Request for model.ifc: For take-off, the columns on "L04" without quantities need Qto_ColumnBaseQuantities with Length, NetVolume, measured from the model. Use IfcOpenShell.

First a look at what the model holds.

```python
import ifcopenshell
import ifcopenshell.util.element
import ifcopenshell.util.unit

model = ifcopenshell.open("model.ifc")
print(model.schema)
for unit_type in ("LENGTHUNIT", "AREAUNIT", "VOLUMEUNIT"):
    print(unit_type, ifcopenshell.util.unit.calculate_unit_scale(model, unit_type))
storey = next(s for s in model.by_type("IfcBuildingStorey") if s.Name == "L04")
columns = [e for e in ifcopenshell.util.element.get_decomposition(storey) if e.is_a("IfcColumn")]
for e in sorted(columns, key=lambda e: e.id()):
    print(e.id(), e.is_a(), e.Name, list(ifcopenshell.util.element.get_psets(e, qtos_only=True)), sep=" | ")
```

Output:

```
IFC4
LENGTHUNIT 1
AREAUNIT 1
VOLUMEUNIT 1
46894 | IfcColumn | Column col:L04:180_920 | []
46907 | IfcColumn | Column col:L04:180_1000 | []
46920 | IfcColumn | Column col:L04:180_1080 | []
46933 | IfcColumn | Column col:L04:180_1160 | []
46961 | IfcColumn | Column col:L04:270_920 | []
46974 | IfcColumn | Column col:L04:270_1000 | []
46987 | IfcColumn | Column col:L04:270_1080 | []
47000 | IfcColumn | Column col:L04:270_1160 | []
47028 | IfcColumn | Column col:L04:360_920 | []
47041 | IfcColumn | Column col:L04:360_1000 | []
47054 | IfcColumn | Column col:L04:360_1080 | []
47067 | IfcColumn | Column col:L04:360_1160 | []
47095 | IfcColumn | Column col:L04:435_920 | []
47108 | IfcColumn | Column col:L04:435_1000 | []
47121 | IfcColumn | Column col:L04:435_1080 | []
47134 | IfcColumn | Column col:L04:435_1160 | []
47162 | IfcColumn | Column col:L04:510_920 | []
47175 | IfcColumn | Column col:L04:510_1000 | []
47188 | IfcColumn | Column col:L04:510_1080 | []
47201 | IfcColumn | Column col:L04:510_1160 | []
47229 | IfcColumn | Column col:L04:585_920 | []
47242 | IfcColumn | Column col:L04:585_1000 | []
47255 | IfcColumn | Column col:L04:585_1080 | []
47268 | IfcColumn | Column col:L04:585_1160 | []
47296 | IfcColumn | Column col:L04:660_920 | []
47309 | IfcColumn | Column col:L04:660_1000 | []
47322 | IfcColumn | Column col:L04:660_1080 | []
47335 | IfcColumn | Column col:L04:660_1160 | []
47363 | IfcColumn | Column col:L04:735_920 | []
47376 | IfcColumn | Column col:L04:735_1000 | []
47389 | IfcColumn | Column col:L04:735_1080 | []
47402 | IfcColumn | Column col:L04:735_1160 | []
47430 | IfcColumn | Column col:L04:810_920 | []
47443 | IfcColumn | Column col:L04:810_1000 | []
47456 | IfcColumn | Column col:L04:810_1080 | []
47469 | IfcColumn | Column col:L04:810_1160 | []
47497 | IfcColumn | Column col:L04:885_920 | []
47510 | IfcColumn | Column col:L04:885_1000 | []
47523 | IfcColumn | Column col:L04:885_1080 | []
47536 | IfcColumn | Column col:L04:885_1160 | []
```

```python
import ifcopenshell
import ifcopenshell.api.pset
import ifcopenshell.geom
import ifcopenshell.util.element
import ifcopenshell.util.shape
import ifcopenshell.util.unit

model = ifcopenshell.open("model.ifc")
unit_scale = ifcopenshell.util.unit.calculate_unit_scale(model)
volume_scale = ifcopenshell.util.unit.calculate_unit_scale(model, "VOLUMEUNIT")
settings = ifcopenshell.geom.settings()

storey = next(s for s in model.by_type("IfcBuildingStorey") if s.Name == "L04")
columns = [e for e in ifcopenshell.util.element.get_decomposition(storey) if e.is_a("IfcColumn")]

for e in sorted(columns, key=lambda e: e.id()):
    if ifcopenshell.util.element.get_psets(e, qtos_only=True, should_inherit=False):
        continue
    # Geometry comes back in metres, in the element's own axes.
    shape = ifcopenshell.geom.create_shape(settings, e)
    values = {
        "Length": ifcopenshell.util.shape.get_z(shape.geometry) / unit_scale,
        "NetVolume": ifcopenshell.util.shape.get_volume(shape.geometry) / volume_scale,
    }
    qto = ifcopenshell.api.pset.add_qto(model, product=e, name="Qto_ColumnBaseQuantities")
    ifcopenshell.api.pset.edit_qto(model, qto=qto, properties=values)
    print(e.id(), {k: round(v, 3) for k, v in values.items()})

model.write("model-out.ifc")
```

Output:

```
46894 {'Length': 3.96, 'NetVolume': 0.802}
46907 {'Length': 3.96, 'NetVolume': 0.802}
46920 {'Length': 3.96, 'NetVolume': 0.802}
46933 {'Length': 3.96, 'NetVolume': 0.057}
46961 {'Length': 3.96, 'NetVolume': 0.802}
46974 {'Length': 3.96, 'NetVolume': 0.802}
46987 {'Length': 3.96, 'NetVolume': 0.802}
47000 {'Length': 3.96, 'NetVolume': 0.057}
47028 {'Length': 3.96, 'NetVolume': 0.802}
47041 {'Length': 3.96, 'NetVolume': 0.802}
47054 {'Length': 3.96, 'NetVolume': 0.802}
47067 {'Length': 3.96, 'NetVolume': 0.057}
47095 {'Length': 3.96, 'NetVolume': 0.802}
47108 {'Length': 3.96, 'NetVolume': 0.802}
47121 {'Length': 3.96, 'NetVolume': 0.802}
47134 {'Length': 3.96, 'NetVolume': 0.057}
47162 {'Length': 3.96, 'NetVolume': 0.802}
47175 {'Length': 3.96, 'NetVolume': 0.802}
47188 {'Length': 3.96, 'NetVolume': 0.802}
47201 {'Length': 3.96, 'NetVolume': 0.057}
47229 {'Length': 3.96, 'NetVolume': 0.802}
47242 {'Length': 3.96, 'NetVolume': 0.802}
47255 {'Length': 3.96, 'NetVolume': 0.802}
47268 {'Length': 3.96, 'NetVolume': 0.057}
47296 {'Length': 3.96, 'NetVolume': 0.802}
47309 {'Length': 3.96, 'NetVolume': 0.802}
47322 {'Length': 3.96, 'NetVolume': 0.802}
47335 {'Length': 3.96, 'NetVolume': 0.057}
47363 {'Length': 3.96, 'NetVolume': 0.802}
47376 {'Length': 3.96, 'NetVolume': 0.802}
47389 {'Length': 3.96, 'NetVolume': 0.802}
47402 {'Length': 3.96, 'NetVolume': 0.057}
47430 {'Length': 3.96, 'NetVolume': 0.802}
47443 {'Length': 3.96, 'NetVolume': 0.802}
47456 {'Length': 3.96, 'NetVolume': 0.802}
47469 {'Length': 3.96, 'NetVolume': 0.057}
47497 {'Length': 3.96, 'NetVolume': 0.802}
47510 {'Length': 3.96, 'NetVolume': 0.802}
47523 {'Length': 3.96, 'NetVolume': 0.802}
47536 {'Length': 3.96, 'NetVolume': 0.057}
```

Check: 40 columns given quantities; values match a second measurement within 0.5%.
